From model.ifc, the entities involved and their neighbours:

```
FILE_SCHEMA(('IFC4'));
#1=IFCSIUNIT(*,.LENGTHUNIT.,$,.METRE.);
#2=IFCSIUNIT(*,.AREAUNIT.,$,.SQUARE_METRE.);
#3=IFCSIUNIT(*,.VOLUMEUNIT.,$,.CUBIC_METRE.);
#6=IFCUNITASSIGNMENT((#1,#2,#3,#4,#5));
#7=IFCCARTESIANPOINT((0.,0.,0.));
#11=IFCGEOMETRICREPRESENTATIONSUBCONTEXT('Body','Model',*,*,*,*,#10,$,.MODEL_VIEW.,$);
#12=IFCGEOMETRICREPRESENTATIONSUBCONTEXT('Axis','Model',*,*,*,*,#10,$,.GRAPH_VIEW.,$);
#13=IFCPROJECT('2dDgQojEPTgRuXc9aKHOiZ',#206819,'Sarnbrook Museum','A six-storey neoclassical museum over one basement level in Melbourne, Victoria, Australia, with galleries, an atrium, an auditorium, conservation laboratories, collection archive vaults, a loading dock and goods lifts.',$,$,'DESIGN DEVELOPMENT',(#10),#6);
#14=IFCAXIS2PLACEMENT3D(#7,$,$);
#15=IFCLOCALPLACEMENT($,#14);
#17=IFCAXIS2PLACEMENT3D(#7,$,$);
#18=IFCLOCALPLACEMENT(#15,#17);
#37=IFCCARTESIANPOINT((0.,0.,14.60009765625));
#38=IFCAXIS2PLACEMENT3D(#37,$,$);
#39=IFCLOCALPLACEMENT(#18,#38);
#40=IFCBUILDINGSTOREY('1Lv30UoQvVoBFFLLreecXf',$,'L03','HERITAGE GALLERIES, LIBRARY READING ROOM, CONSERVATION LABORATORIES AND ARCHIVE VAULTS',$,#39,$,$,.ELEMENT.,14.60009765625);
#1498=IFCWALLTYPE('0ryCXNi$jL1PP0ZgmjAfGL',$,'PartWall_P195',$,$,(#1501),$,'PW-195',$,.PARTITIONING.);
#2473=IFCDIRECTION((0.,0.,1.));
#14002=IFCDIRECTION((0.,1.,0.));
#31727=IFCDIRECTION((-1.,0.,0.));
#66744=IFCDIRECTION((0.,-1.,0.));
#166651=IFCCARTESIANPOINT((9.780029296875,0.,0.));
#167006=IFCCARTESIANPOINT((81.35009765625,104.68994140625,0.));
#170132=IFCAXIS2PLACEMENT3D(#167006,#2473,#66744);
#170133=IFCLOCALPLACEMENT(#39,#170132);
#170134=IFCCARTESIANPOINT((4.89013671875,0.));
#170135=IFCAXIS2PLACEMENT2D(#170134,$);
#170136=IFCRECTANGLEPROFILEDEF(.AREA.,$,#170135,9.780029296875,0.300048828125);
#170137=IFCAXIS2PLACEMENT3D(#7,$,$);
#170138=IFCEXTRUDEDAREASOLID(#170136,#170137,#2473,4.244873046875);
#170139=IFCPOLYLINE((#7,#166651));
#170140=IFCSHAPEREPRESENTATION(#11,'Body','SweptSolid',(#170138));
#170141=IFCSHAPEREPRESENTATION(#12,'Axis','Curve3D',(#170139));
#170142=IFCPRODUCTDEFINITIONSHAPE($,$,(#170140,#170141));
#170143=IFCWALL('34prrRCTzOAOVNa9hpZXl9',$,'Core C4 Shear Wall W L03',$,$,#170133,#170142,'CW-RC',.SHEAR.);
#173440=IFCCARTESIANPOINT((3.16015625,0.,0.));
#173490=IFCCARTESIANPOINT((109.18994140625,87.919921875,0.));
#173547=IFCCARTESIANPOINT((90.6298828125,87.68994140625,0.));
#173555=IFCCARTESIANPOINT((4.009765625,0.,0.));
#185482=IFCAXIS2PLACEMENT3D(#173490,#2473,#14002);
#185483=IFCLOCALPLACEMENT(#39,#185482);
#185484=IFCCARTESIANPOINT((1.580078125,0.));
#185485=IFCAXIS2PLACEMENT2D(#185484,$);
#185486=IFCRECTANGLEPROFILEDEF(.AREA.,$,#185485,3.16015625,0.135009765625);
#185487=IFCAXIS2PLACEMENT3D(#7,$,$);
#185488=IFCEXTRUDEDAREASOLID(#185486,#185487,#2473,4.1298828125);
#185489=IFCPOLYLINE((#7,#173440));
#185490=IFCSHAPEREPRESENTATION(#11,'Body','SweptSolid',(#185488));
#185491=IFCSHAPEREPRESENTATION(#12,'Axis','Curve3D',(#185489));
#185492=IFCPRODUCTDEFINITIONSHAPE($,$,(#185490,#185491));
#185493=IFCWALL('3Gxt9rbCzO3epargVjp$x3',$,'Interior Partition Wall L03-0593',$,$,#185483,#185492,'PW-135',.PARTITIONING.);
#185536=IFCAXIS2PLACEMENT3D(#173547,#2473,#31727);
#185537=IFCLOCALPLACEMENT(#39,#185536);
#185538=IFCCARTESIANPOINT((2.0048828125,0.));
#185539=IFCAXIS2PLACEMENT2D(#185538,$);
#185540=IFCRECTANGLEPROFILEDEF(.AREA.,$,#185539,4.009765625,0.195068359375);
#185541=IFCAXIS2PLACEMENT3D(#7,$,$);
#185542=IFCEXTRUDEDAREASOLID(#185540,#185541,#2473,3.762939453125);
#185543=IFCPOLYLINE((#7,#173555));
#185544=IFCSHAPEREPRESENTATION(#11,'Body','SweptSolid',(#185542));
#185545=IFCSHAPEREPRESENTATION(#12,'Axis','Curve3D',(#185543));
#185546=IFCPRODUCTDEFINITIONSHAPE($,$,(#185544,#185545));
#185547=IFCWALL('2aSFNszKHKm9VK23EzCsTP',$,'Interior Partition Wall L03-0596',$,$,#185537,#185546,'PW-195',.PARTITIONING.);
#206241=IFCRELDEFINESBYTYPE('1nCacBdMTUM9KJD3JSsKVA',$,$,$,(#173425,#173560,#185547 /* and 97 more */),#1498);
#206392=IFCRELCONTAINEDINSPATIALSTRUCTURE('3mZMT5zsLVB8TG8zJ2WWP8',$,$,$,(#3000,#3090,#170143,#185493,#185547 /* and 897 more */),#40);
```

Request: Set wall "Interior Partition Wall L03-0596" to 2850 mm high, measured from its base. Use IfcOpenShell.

```python
import ifcopenshell
import ifcopenshell.geom
import ifcopenshell.util.representation
import ifcopenshell.util.shape

model = ifcopenshell.open("model.ifc")
settings = ifcopenshell.geom.settings()


def volume(element):
    """Net volume in cubic metres, openings subtracted."""
    shape = ifcopenshell.geom.create_shape(settings, element)
    return ifcopenshell.util.shape.get_volume(shape.geometry)


wall = model.by_id(185547)
before = volume(wall)

body = ifcopenshell.util.representation.get_representation(wall, "Model", "Body")
solid = body.Items[0]
old_height = solid.Depth
solid.Depth = 2.85
after = volume(wall)

print(f"height {old_height:g} -> {solid.Depth:g}, volume {before:.3f} -> {after:.3f} m3")

model.write("model_v2.ifc")
```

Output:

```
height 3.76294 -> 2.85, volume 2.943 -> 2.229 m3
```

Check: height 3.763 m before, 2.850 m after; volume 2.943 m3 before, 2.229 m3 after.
